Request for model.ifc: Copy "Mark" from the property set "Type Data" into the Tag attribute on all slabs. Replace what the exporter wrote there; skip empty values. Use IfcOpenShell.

First a look at what the model holds.

```python
import ifcopenshell
import ifcopenshell.util.element

model = ifcopenshell.open("model.ifc")
print(model.schema)
slabs = model.by_type("IfcSlab")
print(len(slabs), "slabs")
for e in slabs[:8]:
    source = ifcopenshell.util.element.get_pset(e, "Type Data", "Mark")
    target = e.Tag
    print(e.id(), repr(source), repr(target), sep=" | ")
```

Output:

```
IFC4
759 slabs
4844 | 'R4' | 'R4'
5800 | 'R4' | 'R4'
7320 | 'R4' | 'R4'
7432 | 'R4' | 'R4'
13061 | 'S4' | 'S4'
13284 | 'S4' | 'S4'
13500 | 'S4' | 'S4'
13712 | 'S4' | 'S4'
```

```python
import ifcopenshell
import ifcopenshell.util.element

model = ifcopenshell.open("model.ifc")

count = 0
for e in model.by_type("IfcSlab"):
    value = ifcopenshell.util.element.get_pset(e, "Type Data", "Mark")
    current = e.Tag
    if not value or not value.strip() or current == value:
        continue
    e.Tag = value
    count += 1

print(count, "slabs updated")

model.write("model_v2.ifc")
```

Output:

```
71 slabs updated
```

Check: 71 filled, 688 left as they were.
